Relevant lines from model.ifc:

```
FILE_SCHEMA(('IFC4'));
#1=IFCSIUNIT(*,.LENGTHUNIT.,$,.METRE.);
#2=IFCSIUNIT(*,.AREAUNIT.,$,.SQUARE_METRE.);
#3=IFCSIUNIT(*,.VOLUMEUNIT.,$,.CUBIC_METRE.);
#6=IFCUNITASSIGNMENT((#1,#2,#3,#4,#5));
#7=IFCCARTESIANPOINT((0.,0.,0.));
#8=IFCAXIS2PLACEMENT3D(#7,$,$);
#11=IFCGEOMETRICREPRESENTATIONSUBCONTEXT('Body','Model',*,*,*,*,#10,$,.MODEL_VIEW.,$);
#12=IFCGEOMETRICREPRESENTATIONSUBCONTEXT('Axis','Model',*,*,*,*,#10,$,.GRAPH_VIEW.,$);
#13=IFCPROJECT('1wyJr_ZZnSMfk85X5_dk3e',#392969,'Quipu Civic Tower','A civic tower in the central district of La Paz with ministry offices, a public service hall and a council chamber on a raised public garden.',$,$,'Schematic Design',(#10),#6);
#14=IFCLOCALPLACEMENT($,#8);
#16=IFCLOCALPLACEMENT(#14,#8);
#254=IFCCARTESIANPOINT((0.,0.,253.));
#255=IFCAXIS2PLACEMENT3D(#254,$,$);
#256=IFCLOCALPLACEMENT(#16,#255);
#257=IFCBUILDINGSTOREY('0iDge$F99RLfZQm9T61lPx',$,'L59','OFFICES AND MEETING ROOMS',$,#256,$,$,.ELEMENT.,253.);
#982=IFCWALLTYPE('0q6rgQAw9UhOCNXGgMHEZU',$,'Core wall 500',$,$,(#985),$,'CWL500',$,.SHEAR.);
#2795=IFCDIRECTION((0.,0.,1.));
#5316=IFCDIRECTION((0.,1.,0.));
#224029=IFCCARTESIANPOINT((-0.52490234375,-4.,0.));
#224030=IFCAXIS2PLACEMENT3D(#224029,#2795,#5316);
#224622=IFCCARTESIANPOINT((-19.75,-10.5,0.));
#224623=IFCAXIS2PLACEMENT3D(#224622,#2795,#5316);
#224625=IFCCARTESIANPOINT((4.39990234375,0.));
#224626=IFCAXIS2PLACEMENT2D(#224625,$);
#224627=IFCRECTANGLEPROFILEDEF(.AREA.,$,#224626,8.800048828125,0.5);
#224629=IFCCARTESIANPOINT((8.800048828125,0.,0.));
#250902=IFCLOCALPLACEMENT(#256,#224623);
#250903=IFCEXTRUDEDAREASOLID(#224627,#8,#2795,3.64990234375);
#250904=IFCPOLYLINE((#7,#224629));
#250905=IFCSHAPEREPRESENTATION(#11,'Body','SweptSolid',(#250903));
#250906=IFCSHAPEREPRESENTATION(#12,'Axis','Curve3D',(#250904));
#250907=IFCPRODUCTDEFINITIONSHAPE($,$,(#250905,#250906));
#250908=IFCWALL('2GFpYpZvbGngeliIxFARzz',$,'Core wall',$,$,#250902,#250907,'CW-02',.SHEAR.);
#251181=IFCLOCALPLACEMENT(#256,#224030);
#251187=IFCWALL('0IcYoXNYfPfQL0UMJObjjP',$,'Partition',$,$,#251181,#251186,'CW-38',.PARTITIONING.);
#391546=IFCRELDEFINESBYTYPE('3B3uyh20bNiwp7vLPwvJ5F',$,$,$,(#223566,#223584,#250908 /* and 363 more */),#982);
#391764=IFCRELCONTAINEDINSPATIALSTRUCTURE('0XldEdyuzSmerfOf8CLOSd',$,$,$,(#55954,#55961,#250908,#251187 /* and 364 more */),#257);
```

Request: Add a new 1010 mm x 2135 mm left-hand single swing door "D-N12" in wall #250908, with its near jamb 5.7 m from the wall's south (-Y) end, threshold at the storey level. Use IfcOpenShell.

```python
import numpy as np
import ifcopenshell
import ifcopenshell.api.feature
import ifcopenshell.api.geometry
import ifcopenshell.api.root
import ifcopenshell.api.spatial
import ifcopenshell.geom
import ifcopenshell.util.element
import ifcopenshell.util.placement
import ifcopenshell.util.representation
import ifcopenshell.util.shape
import ifcopenshell.util.unit

model = ifcopenshell.open("model.ifc")
unit_scale = ifcopenshell.util.unit.calculate_unit_scale(model)
settings = ifcopenshell.geom.settings()


def volume(element):
    """Net volume in cubic metres, openings subtracted."""
    shape = ifcopenshell.geom.create_shape(settings, element)
    return ifcopenshell.util.shape.get_volume(shape.geometry)


wall = model.by_guid("2GFpYpZvbGngeliIxFARzz")
storey = ifcopenshell.util.element.get_container(wall, ifc_class="IfcBuildingStorey")
context = ifcopenshell.util.representation.get_context(model, "Model", "Body", "MODEL_VIEW")
before = volume(wall)

width, height, from_end, sill = 1.01, 2.135, 5.7, 0.0  # metres

# The wall runs along its own X axis, and the end named is its -X end.
wall_shape = ifcopenshell.geom.create_shape(settings, wall)
x, y, z = ifcopenshell.util.shape.get_vertices(wall_shape.geometry).T
start = x.min() + from_end
face, thickness = float(y.min()), float(y.max() - y.min())
wall_matrix = ifcopenshell.util.placement.get_local_placement(wall.ObjectPlacement)
level = ifcopenshell.util.placement.get_local_placement(storey.ObjectPlacement)[2, 3]


def in_wall(x, y):
    """Placement at x, y metres in the wall's axes, at sill height."""
    matrix = wall_matrix.copy()
    matrix[:, 3] = wall_matrix @ np.array([x / unit_scale, y / unit_scale, 0.0, 1.0])
    matrix[2, 3] = level + sill / unit_scale
    return matrix


# Opening: a box that overshoots both wall faces by 50 mm.
opening = ifcopenshell.api.root.create_entity(model, ifc_class="IfcOpeningElement", predefined_type="OPENING")
box = ifcopenshell.api.geometry.add_wall_representation(
    model, context=context, length=width, height=height, thickness=thickness + 0.1
)
ifcopenshell.api.geometry.assign_representation(model, product=opening, representation=box)
ifcopenshell.api.geometry.edit_object_placement(model, product=opening, matrix=in_wall(start, face - 0.05), is_si=False)
ifcopenshell.api.feature.add_feature(model, feature=opening, element=wall)

door = ifcopenshell.api.root.create_entity(model, ifc_class="IfcDoor", name="D-N12", predefined_type="DOOR")
door.OverallWidth, door.OverallHeight = width / unit_scale, height / unit_scale
door.OperationType = "SINGLE_SWING_LEFT"
body = ifcopenshell.api.geometry.add_door_representation(
    model,
    context=context,
    overall_width=door.OverallWidth,
    overall_height=door.OverallHeight,
    operation_type="SINGLE_SWING_LEFT",
    lining_properties={"LiningDepth": thickness / unit_scale, "ThresholdDepth": thickness / unit_scale},
)
ifcopenshell.api.geometry.assign_representation(model, product=door, representation=body)
ifcopenshell.api.spatial.assign_container(model, products=[door], relating_structure=storey)
ifcopenshell.api.feature.add_filling(model, opening=opening, element=door)

# The lining spans the wall, so the door starts at the wall face.
ifcopenshell.api.geometry.edit_object_placement(model, product=door, matrix=in_wall(start, face), is_si=False)

after = volume(wall)

print(f"wall volume {before:.3f} -> {after:.3f} m3")

model.write("model_edited.ifc")
```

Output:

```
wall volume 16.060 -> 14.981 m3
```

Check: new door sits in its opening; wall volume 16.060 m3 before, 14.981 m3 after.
